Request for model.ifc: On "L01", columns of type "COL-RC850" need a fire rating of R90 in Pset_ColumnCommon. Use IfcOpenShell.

First a look at what the model holds.

```python
import ifcopenshell
import ifcopenshell.util.element

model = ifcopenshell.open("model.ifc")
print(model.schema)
storey = next(s for s in model.by_type("IfcBuildingStorey") if s.Name == "L01")
columns = [e for e in ifcopenshell.util.element.get_decomposition(storey) if e.is_a("IfcColumn")]
seen = {}
for e in columns:
    element_type = ifcopenshell.util.element.get_type(e)
    key = (element_type.Name if element_type != e and element_type else None, ifcopenshell.util.element.get_pset(e, "Pset_ColumnCommon", "FireRating"))
    seen[key] = seen.get(key, 0) + 1
for (name, value), count in sorted(seen.items(), key=str):
    print(count, "x", name, "|", value)
```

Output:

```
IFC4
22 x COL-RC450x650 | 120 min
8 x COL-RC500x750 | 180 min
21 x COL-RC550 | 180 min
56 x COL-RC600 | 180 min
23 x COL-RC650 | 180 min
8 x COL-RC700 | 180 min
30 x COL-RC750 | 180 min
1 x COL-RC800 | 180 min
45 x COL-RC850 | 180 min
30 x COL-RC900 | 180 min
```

```python
import ifcopenshell
import ifcopenshell.api.pset
import ifcopenshell.util.element

model = ifcopenshell.open("model.ifc")

storey = next(s for s in model.by_type("IfcBuildingStorey") if s.Name == "L01")
columns = [e for e in ifcopenshell.util.element.get_decomposition(storey) if e.is_a("IfcColumn")]

count = 0
for e in columns:
    element_type = ifcopenshell.util.element.get_type(e)
    if element_type in (None, e) or element_type.Name != "COL-RC850":
        continue
    # add_pset returns the element's existing set when there is one.
    pset = ifcopenshell.api.pset.add_pset(model, product=e, name="Pset_ColumnCommon")
    ifcopenshell.api.pset.edit_pset(model, pset=pset, properties={"FireRating": "R90"})
    count += 1

print(count, "columns updated")

model.write("model_edited.ifc")
```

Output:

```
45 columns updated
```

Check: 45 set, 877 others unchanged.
